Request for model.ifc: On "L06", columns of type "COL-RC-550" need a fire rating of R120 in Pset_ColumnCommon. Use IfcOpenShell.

First a look at what the model holds.

```python
import ifcopenshell
import ifcopenshell.util.element

model = ifcopenshell.open("model.ifc")
print(model.schema)
storey = next(s for s in model.by_type("IfcBuildingStorey") if s.Name == "L06")
columns = [e for e in ifcopenshell.util.element.get_decomposition(storey) if e.is_a("IfcColumn")]
seen = {}
for e in columns:
    element_type = ifcopenshell.util.element.get_type(e)
    key = (element_type.Name if element_type != e and element_type else None, ifcopenshell.util.element.get_pset(e, "Pset_ColumnCommon", "FireRating"))
    seen[key] = seen.get(key, 0) + 1
for (name, value), count in sorted(seen.items(), key=str):
    print(count, "x", name, "|", value)
```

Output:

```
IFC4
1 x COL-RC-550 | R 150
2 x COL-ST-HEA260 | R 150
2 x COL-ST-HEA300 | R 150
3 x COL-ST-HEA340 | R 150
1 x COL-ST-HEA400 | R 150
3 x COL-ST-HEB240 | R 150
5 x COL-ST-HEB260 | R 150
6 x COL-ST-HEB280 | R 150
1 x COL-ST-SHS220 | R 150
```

```python
import ifcopenshell
import ifcopenshell.api.pset
import ifcopenshell.util.element

model = ifcopenshell.open("model.ifc")

storey = next(s for s in model.by_type("IfcBuildingStorey") if s.Name == "L06")
columns = [e for e in ifcopenshell.util.element.get_decomposition(storey) if e.is_a("IfcColumn")]

count = 0
for e in columns:
    element_type = ifcopenshell.util.element.get_type(e)
    if element_type in (None, e) or element_type.Name != "COL-RC-550":
        continue
    # add_pset returns the element's existing set when there is one.
    pset = ifcopenshell.api.pset.add_pset(model, product=e, name="Pset_ColumnCommon")
    ifcopenshell.api.pset.edit_pset(model, pset=pset, properties={"FireRating": "R120"})
    count += 1

print(count, "columns updated")

model.write("model_rev.ifc")
```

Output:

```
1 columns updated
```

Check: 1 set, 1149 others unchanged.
